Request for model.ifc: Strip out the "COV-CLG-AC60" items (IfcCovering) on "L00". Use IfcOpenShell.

First a look at what the model holds.

```python
import ifcopenshell
import ifcopenshell.util.element

model = ifcopenshell.open("model.ifc")
print(model.schema)
storey = next(s for s in model.by_type("IfcBuildingStorey") if s.Name == "L00")
coverings = [e for e in ifcopenshell.util.element.get_decomposition(storey) if e.is_a("IfcCovering")]
seen = {}
for e in coverings:
    element_type = ifcopenshell.util.element.get_type(e)
    name = element_type.Name if element_type not in (None, e) else None
    seen[name] = seen.get(name, 0) + 1
for name, count in sorted(seen.items(), key=str):
    print(count, "x", name)
```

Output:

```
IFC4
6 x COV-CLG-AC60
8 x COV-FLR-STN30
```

```python
import ifcopenshell
import ifcopenshell.api.root
import ifcopenshell.util.element

model = ifcopenshell.open("model.ifc")

storey = next(s for s in model.by_type("IfcBuildingStorey") if s.Name == "L00")
coverings = [e for e in ifcopenshell.util.element.get_decomposition(storey) if e.is_a("IfcCovering")]
targets = [e for e in coverings if (t := ifcopenshell.util.element.get_type(e)) not in (None, e) and t.Name == "COV-CLG-AC60"]

for e in targets:
    ifcopenshell.api.root.remove_product(model, product=e)
print(len(targets), "removed")

model.write("model_rev.ifc")
```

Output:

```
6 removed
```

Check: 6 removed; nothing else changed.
